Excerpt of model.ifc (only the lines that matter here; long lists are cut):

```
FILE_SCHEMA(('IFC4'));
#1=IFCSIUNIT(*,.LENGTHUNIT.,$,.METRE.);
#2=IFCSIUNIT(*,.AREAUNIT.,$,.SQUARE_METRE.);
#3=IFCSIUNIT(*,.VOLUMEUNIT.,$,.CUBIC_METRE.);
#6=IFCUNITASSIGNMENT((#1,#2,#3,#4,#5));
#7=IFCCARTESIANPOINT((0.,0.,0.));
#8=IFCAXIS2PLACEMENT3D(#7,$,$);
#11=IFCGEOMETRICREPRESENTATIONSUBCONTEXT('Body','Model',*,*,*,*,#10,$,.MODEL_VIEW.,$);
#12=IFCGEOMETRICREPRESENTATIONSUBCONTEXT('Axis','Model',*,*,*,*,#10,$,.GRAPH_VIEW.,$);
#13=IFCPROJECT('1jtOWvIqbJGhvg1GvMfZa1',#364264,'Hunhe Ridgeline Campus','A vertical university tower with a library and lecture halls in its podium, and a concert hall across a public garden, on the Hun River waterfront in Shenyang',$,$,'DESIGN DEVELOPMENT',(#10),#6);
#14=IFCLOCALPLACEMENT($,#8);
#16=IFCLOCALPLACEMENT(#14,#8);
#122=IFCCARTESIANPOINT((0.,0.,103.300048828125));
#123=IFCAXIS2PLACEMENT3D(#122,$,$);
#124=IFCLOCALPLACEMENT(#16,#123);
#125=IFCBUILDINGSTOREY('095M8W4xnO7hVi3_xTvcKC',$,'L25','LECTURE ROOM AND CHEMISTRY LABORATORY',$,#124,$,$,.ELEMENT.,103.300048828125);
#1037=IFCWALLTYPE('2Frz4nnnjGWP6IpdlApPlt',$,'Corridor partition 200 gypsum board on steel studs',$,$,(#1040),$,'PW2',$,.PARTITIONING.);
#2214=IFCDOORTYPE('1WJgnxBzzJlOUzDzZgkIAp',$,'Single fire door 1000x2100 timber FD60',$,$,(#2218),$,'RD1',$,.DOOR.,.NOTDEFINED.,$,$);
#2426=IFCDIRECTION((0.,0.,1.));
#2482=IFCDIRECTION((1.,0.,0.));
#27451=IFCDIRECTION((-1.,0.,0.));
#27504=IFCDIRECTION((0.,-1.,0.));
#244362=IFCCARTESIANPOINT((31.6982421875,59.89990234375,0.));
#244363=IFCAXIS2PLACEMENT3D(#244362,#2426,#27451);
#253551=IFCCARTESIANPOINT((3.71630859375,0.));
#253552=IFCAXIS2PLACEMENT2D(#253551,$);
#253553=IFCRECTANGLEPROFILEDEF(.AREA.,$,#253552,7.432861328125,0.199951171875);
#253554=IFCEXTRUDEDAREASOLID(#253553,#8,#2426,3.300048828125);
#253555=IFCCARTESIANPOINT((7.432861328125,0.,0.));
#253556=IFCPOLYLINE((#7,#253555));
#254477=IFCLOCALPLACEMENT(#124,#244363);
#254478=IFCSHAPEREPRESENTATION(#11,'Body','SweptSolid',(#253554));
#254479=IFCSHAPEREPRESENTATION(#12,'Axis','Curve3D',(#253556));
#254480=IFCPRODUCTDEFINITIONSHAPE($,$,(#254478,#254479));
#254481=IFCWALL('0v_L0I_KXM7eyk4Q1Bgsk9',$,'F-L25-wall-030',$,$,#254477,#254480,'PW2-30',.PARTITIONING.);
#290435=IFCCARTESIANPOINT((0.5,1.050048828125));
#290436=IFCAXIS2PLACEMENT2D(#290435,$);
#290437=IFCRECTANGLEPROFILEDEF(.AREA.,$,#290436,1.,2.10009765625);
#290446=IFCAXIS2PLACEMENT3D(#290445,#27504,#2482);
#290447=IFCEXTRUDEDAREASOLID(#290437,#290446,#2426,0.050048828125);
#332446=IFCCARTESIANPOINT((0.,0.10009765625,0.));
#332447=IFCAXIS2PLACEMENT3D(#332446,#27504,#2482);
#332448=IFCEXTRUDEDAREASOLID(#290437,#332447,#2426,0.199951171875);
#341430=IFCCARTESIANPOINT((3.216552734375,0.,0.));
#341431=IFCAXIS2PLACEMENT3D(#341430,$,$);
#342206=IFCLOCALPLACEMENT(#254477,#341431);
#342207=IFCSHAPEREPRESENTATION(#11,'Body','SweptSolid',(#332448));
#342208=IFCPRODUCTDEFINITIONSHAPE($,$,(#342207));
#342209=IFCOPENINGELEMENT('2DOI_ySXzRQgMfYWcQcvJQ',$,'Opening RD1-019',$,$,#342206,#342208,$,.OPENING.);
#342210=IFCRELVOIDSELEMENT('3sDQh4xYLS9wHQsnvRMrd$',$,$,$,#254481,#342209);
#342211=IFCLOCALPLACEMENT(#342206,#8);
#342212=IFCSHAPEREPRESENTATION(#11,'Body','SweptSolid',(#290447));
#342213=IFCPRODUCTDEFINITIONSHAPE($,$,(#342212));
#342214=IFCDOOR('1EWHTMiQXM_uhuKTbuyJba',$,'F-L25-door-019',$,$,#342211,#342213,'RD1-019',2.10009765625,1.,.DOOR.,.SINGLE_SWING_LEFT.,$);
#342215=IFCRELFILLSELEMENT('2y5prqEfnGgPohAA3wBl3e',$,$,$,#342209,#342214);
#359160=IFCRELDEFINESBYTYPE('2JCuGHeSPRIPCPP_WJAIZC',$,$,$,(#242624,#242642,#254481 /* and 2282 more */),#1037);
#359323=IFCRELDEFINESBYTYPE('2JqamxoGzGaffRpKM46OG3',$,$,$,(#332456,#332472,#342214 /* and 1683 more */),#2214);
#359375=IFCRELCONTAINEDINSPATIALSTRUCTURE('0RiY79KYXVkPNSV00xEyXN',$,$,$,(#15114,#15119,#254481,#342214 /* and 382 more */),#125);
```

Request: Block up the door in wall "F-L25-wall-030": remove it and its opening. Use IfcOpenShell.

```python
import ifcopenshell
import ifcopenshell.api.feature
import ifcopenshell.api.root
import ifcopenshell.geom
import ifcopenshell.util.shape

model = ifcopenshell.open("model.ifc")
settings = ifcopenshell.geom.settings()


def volume(element):
    """Net volume in cubic metres, openings subtracted."""
    shape = ifcopenshell.geom.create_shape(settings, element)
    return ifcopenshell.util.shape.get_volume(shape.geometry)


door = model.by_guid("1EWHTMiQXM_uhuKTbuyJba")
opening = door.FillsVoids[0].RelatingOpeningElement
wall = opening.VoidsElements[0].RelatingBuildingElement
before = volume(wall)

ifcopenshell.api.root.remove_product(model, product=door)
ifcopenshell.api.feature.remove_feature(model, feature=opening)

after = volume(wall)

print(f"wall volume {before:.3f} -> {after:.3f} m3")

model.write("model_edited.ifc")
```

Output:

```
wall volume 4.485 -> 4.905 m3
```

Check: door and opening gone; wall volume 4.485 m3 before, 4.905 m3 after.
